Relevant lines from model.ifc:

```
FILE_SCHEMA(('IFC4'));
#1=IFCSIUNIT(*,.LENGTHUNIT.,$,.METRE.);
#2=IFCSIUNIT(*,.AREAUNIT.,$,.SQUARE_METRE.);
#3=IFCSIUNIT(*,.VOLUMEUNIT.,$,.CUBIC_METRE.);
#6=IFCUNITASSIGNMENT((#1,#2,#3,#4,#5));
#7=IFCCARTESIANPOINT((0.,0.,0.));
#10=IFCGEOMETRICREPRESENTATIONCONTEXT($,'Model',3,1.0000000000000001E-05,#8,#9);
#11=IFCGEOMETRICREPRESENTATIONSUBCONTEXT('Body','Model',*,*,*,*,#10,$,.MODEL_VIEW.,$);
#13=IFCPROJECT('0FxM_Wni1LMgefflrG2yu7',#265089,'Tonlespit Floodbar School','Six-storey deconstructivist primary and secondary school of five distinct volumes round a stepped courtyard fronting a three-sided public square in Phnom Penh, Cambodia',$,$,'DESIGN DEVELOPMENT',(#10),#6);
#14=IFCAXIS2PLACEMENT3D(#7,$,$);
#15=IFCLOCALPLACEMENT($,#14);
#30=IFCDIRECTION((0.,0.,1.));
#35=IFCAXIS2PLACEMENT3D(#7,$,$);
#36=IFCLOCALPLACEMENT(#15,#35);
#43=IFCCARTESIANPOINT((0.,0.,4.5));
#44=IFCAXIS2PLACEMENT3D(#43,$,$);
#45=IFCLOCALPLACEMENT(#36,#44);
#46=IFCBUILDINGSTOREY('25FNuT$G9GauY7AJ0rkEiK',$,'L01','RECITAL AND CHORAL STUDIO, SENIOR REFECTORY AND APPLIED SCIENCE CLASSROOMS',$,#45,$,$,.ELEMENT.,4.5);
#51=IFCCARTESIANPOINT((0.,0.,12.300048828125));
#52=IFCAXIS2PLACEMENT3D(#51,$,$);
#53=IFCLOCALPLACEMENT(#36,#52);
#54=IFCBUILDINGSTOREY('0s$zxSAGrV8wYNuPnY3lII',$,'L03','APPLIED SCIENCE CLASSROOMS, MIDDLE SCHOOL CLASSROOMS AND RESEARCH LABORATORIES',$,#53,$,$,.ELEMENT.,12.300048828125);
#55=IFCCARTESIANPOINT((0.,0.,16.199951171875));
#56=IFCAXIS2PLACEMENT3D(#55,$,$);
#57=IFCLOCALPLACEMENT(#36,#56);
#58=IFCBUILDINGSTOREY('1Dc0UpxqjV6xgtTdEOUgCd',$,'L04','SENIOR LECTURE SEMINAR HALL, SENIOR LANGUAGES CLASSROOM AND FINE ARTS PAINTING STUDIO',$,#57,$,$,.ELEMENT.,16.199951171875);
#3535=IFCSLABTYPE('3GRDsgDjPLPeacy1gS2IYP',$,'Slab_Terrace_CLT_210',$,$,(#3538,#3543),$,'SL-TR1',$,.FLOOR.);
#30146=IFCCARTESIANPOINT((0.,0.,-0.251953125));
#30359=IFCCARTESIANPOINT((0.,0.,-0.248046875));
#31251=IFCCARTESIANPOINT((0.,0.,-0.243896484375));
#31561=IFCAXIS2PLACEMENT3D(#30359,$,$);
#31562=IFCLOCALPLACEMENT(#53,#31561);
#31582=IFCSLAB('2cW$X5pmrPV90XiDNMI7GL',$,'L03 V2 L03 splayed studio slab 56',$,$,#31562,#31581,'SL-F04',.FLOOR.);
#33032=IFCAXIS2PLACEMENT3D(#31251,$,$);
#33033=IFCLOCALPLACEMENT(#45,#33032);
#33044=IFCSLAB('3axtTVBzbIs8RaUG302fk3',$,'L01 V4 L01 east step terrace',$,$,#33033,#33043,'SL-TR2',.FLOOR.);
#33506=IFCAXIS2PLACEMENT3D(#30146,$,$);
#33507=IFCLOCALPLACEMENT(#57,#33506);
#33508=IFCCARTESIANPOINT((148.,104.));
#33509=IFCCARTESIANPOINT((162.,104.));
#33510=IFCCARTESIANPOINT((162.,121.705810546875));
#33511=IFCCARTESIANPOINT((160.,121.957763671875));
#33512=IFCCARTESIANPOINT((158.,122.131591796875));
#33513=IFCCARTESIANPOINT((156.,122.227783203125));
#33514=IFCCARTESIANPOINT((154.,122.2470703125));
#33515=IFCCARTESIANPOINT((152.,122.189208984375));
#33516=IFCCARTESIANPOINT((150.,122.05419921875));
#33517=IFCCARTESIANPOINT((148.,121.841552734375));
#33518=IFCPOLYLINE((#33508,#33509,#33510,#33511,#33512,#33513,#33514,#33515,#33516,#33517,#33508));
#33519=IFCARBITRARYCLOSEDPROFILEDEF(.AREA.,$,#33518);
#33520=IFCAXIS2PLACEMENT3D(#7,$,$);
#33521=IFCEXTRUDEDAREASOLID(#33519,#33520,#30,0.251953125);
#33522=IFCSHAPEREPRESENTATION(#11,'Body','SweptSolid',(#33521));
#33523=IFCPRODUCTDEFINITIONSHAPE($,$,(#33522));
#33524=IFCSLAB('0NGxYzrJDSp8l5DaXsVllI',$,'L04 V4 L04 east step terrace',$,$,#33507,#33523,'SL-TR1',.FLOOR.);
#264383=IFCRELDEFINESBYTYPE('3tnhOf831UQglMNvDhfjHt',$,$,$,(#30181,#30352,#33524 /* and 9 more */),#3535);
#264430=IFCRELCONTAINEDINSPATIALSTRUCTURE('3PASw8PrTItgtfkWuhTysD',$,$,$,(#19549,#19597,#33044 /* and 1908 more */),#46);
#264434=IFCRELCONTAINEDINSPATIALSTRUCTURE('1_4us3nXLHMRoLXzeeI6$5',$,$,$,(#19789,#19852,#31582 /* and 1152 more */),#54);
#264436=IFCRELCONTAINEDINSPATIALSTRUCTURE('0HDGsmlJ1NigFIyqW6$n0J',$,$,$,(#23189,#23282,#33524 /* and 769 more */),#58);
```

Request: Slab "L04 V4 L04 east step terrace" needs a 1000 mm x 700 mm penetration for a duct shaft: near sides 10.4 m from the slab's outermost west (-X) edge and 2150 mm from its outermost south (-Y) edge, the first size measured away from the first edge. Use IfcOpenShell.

```python
import numpy as np
import ifcopenshell
import ifcopenshell.api.feature
import ifcopenshell.api.geometry
import ifcopenshell.api.root
import ifcopenshell.geom
import ifcopenshell.util.placement
import ifcopenshell.util.representation
import ifcopenshell.util.shape
import ifcopenshell.util.unit

model = ifcopenshell.open("model.ifc")
unit_scale = ifcopenshell.util.unit.calculate_unit_scale(model)
settings = ifcopenshell.geom.settings()


def volume(element):
    """Net volume in cubic metres, openings subtracted."""
    shape = ifcopenshell.geom.create_shape(settings, element)
    return ifcopenshell.util.shape.get_volume(shape.geometry)


slab = model.by_id(33524)
before = volume(slab)

# Extent in the slab's own axes, in metres. The edges named are its -X and -Y sides.
slab_shape = ifcopenshell.geom.create_shape(settings, slab)
vertices = ifcopenshell.util.shape.get_vertices(slab_shape.geometry)
x_min, y_min, bottom = vertices.min(axis=0)
top = vertices[:, 2].max()

opening = ifcopenshell.api.root.create_entity(model, ifc_class="IfcOpeningElement", name="Duct shaft opening", predefined_type="OPENING")
context = ifcopenshell.util.representation.get_context(model, "Model", "Body", "MODEL_VIEW")
width, depth = 1, 0.7
outline = [(0.0, 0.0), (width, 0.0), (width, depth), (0.0, depth), (0.0, 0.0)]
# Overshoot both faces by 50 mm so the cut is clean.
shape = ifcopenshell.api.geometry.add_slab_representation(
    model, context=context, depth=top - bottom + 0.1, polyline=outline
)
ifcopenshell.api.geometry.assign_representation(model, product=opening, representation=shape)

matrix = ifcopenshell.util.placement.get_local_placement(slab.ObjectPlacement)
matrix[:, 3] = matrix @ np.append(np.array([x_min + 10.4, y_min + 2.15, bottom - 0.05]) / unit_scale, 1.0)
ifcopenshell.api.geometry.edit_object_placement(model, product=opening, matrix=matrix, is_si=False)
ifcopenshell.api.feature.add_feature(model, feature=opening, element=slab)

after = volume(slab)

print(f"slab volume {before:.3f} -> {after:.3f} m3")

model.write("model_edited.ifc")
```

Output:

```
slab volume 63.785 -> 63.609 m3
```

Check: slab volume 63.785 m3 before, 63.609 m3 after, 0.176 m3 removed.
